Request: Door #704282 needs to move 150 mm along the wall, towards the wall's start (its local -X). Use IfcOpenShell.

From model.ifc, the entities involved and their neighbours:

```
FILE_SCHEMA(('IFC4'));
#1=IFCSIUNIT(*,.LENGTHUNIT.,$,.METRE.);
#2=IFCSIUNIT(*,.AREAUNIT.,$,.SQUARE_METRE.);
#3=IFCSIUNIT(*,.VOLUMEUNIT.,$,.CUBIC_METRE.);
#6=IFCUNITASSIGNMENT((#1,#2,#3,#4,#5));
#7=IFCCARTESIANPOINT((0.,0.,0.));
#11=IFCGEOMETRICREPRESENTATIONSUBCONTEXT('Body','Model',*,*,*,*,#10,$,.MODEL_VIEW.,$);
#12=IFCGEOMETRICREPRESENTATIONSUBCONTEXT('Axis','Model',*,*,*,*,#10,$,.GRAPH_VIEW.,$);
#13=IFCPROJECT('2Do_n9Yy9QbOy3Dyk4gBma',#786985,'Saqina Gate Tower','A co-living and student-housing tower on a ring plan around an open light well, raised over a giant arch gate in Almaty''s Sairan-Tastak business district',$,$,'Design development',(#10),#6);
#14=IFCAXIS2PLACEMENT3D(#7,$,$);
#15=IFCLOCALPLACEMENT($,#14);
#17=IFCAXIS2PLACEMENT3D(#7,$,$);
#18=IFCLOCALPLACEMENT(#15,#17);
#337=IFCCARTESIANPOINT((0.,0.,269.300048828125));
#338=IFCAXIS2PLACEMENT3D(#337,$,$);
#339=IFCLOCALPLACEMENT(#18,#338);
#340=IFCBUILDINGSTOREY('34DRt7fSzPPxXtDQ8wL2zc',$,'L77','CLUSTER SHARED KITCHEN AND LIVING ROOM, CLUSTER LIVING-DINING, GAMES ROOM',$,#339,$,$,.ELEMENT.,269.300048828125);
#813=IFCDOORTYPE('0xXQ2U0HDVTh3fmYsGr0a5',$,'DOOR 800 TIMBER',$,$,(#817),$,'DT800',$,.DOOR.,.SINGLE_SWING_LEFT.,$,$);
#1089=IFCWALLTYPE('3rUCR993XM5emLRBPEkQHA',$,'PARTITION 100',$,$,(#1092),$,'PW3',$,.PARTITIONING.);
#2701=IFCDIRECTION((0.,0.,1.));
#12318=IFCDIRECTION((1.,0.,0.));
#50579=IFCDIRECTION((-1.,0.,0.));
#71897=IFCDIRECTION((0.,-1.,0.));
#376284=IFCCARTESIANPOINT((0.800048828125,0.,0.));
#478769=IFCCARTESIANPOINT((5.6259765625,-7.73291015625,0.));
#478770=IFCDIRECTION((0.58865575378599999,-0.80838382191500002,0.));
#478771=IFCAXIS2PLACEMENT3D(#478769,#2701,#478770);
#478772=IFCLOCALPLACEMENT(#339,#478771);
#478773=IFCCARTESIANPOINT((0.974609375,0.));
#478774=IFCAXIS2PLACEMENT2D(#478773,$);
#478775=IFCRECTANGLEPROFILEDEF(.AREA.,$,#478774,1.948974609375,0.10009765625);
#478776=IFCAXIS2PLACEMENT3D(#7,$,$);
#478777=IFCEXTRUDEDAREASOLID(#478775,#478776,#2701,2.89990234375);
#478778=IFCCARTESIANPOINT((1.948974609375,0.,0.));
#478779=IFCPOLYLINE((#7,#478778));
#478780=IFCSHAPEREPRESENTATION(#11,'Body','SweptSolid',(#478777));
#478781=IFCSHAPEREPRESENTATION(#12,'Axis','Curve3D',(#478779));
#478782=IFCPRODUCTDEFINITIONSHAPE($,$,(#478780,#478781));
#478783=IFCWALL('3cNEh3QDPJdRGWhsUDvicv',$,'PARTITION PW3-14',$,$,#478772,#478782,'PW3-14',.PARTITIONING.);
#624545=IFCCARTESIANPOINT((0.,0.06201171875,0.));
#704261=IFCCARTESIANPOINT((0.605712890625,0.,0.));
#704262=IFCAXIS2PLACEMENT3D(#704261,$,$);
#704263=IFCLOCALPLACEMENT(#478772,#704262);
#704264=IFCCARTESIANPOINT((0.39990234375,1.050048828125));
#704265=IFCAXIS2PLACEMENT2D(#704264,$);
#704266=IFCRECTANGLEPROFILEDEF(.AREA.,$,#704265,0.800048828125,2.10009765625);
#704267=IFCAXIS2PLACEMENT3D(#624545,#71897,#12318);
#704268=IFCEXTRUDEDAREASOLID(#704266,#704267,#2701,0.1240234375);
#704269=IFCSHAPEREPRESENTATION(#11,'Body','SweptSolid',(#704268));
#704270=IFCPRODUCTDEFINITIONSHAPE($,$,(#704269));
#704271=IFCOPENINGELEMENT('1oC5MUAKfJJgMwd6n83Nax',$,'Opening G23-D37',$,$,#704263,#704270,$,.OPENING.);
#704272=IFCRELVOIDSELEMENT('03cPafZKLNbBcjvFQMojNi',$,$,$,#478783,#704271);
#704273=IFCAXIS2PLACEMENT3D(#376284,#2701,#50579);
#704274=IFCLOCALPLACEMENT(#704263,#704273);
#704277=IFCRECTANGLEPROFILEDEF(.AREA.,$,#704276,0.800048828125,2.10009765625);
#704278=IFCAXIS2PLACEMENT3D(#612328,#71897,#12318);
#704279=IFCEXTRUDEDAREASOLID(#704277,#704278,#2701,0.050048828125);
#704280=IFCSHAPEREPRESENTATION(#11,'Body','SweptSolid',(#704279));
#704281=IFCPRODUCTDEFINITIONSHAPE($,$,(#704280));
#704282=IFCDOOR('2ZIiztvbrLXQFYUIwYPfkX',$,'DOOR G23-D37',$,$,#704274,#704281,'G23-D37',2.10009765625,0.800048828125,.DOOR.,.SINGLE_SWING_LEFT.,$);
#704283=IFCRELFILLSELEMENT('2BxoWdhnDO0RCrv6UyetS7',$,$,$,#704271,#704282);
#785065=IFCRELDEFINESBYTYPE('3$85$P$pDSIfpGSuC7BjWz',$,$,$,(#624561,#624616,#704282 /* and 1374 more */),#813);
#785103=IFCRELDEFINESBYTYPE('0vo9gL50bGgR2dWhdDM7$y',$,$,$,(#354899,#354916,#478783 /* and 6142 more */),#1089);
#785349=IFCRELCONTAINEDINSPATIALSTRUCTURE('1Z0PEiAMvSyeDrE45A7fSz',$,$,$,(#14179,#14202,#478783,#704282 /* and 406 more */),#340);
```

```python
import ifcopenshell
import ifcopenshell.api.geometry
import ifcopenshell.util.placement

model = ifcopenshell.open("model.ifc")

door = model.by_guid("2ZIiztvbrLXQFYUIwYPfkX")
opening = door.FillsVoids[0].RelatingOpeningElement
wall = opening.VoidsElements[0].RelatingBuildingElement

wall_matrix = ifcopenshell.util.placement.get_local_placement(wall.ObjectPlacement)
shift = wall_matrix[:3, 0] * -0.15
before = ifcopenshell.util.placement.get_local_placement(door.ObjectPlacement)[:3, 3].copy()

# The door is placed relative to its opening, so it follows when the opening moves.
matrix = ifcopenshell.util.placement.get_local_placement(opening.ObjectPlacement)
matrix[:3, 3] += shift
ifcopenshell.api.geometry.edit_object_placement(
    model, product=opening, matrix=matrix, is_si=False, should_transform_children=True
)

after = ifcopenshell.util.placement.get_local_placement(door.ObjectPlacement)[:3, 3]
print("door moved by", (after - before).round(3) + 0.0)

model.write("model_rev.ifc")
```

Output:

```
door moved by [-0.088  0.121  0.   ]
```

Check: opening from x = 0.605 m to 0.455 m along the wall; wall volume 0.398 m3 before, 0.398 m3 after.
